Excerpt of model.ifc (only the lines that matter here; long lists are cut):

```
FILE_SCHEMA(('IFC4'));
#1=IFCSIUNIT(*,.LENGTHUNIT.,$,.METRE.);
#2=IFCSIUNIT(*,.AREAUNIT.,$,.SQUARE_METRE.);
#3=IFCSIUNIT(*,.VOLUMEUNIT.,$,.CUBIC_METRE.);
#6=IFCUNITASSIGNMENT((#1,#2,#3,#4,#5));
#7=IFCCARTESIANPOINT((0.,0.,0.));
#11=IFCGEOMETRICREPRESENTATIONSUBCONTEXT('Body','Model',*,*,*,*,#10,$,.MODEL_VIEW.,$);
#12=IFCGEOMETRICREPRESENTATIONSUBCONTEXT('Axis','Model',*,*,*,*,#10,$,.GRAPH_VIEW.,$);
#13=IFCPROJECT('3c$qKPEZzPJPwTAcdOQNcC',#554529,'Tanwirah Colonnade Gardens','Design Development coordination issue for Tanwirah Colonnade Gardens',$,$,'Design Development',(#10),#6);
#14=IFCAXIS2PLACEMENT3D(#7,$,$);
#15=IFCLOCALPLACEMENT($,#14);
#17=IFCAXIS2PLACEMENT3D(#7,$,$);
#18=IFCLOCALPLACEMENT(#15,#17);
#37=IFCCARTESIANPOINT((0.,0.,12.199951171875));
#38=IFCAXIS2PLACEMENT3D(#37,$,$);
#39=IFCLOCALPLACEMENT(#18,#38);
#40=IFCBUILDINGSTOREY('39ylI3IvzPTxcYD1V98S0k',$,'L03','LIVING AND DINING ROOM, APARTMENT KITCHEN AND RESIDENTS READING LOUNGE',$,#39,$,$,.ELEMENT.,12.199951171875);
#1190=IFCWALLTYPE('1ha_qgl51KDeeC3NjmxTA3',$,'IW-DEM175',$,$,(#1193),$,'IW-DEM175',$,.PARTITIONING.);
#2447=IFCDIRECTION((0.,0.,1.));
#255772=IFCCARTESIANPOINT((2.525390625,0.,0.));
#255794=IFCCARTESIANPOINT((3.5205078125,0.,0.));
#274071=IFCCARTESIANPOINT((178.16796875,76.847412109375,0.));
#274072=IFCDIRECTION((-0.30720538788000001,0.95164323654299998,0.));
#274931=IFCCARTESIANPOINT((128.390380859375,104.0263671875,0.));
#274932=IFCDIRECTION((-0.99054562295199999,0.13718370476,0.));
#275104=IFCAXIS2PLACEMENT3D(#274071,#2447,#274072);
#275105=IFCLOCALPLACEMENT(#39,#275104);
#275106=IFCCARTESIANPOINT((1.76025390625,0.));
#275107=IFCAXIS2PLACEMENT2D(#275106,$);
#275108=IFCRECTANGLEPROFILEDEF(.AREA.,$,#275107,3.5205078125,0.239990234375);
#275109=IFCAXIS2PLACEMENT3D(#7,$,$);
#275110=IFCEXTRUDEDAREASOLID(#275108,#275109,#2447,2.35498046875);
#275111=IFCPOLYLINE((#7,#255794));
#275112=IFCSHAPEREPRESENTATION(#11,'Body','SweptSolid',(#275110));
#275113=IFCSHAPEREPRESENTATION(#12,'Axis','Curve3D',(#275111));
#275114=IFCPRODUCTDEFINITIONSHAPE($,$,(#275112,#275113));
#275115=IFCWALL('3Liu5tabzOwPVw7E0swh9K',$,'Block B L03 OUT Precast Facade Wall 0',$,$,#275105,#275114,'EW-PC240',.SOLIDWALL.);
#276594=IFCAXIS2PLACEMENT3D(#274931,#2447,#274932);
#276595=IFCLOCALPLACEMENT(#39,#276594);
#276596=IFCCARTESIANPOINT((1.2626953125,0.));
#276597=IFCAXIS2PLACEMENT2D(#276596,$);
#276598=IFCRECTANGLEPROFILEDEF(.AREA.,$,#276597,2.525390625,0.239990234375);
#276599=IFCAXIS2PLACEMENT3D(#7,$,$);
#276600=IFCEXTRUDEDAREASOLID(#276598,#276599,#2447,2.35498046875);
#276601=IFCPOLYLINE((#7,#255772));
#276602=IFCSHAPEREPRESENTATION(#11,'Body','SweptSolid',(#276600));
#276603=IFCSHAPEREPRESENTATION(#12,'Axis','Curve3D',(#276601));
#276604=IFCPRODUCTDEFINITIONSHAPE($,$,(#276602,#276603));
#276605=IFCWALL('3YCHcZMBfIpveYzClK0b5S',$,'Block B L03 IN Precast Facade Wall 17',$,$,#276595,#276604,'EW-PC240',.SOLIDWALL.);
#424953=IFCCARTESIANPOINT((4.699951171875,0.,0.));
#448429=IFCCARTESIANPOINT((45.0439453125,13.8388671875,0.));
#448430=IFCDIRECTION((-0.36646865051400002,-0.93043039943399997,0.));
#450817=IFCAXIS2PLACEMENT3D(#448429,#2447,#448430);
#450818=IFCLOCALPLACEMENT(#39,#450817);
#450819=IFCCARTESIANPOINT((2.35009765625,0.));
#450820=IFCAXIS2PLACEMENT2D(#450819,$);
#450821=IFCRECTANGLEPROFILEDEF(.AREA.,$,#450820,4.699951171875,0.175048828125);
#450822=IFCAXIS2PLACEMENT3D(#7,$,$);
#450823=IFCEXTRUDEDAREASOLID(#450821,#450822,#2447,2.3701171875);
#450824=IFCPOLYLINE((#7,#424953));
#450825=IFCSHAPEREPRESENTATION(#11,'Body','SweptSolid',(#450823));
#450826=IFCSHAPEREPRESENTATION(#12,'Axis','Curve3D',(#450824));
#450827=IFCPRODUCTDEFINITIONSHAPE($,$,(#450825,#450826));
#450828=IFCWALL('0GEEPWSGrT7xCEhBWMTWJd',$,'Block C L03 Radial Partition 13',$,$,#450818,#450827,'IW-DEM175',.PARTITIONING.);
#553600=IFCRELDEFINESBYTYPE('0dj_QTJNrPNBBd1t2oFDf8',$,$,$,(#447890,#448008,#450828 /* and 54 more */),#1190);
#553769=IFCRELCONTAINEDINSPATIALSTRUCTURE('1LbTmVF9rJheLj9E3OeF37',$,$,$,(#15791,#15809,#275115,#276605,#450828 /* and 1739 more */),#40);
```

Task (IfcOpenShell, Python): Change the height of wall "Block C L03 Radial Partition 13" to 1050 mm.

```python
import ifcopenshell
import ifcopenshell.geom
import ifcopenshell.util.representation
import ifcopenshell.util.shape
import ifcopenshell.util.unit

model = ifcopenshell.open("model.ifc")
unit_scale = ifcopenshell.util.unit.calculate_unit_scale(model)
settings = ifcopenshell.geom.settings()


def volume(element):
    """Net volume in cubic metres, openings subtracted."""
    shape = ifcopenshell.geom.create_shape(settings, element)
    return ifcopenshell.util.shape.get_volume(shape.geometry)


wall = model.by_guid("0GEEPWSGrT7xCEhBWMTWJd")
before = volume(wall)

body = ifcopenshell.util.representation.get_representation(wall, "Model", "Body")
solid = body.Items[0]
old_height = solid.Depth
solid.Depth = 1.05 / unit_scale
after = volume(wall)

print(f"height {old_height:g} -> {solid.Depth:g}, volume {before:.3f} -> {after:.3f} m3")

model.write("model-out.ifc")
```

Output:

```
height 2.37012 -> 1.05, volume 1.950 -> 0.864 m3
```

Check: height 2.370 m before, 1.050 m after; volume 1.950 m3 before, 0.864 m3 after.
